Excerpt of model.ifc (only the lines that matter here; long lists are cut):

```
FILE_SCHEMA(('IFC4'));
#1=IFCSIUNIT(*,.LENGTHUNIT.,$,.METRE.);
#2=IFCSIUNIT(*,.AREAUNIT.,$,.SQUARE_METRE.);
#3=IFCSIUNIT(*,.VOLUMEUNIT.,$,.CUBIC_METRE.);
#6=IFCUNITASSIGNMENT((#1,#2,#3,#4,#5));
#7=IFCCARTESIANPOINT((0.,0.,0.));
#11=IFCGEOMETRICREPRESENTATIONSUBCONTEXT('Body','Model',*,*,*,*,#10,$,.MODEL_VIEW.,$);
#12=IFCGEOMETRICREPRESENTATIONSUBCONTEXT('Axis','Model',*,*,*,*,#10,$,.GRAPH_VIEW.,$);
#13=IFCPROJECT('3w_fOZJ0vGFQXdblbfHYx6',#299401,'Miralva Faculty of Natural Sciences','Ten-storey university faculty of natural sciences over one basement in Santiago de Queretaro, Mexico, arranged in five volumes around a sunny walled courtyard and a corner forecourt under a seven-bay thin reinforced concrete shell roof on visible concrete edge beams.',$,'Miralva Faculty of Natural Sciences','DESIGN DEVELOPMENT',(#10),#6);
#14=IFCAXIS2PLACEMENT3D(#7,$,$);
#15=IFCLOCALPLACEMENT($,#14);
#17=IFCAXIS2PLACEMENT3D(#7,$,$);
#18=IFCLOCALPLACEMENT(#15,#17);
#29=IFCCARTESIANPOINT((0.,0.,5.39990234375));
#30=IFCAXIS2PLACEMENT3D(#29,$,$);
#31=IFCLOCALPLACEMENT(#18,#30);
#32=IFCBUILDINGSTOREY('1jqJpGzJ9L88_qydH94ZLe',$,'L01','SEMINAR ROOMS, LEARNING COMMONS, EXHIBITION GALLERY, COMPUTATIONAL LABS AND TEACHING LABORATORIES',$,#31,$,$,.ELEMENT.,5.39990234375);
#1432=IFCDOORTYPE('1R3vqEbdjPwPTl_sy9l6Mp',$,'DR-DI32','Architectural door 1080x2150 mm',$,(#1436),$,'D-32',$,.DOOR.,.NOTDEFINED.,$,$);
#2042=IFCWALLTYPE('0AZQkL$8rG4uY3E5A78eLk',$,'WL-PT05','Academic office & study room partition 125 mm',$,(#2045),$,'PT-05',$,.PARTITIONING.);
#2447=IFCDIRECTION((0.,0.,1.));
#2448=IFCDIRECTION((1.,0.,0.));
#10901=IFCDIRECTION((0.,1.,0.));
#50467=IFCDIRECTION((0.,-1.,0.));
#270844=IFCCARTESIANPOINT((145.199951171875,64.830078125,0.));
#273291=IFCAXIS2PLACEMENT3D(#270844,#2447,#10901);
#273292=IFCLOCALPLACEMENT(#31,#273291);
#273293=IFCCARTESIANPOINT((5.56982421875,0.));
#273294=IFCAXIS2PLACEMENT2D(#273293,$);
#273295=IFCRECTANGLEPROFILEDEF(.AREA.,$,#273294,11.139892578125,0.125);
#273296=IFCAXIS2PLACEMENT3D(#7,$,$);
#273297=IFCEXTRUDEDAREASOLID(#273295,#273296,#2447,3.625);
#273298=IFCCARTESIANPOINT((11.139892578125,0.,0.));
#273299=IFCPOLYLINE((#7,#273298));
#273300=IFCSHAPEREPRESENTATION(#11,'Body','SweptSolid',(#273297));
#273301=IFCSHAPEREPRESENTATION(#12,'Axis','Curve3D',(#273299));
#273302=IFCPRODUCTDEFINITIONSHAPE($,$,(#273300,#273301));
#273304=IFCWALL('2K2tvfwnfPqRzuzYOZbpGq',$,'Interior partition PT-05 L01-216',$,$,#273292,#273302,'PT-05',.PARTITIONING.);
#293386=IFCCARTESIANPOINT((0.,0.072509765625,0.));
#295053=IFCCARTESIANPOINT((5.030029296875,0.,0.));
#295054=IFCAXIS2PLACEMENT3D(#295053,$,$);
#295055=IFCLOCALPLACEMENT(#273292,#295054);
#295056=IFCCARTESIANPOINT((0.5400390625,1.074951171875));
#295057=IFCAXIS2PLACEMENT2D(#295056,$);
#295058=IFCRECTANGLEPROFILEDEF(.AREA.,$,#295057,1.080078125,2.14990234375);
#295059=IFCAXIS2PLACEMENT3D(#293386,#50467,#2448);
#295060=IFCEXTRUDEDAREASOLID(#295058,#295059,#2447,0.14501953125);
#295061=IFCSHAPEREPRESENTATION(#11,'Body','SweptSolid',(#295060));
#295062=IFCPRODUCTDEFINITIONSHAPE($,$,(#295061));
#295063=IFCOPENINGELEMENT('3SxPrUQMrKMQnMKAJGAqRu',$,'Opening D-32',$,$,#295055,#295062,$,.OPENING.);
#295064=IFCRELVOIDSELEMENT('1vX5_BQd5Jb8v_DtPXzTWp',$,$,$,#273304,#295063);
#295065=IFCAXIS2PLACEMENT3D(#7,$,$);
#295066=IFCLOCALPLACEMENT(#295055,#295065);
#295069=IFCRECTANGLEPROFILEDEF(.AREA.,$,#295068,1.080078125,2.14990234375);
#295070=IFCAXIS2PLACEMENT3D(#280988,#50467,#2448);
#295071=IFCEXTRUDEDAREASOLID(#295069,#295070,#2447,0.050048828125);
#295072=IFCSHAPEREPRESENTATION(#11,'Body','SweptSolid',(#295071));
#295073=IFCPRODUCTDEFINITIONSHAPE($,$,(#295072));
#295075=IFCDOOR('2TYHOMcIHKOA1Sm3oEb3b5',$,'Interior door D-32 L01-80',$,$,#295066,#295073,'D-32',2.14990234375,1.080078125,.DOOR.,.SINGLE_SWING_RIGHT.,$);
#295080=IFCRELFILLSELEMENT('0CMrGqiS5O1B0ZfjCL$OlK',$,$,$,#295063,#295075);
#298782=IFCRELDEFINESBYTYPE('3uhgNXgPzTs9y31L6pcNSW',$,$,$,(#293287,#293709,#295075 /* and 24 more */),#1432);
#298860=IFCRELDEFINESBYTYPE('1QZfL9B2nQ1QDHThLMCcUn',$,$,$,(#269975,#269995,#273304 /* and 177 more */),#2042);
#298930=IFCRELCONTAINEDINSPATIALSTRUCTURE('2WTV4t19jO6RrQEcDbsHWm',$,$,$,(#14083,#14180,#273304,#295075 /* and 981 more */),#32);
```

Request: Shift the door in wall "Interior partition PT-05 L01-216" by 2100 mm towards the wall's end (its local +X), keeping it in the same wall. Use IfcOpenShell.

```python
import ifcopenshell
import ifcopenshell.api.geometry
import ifcopenshell.util.placement
import ifcopenshell.util.unit

model = ifcopenshell.open("model.ifc")
unit_scale = ifcopenshell.util.unit.calculate_unit_scale(model)

door = model.by_guid("2TYHOMcIHKOA1Sm3oEb3b5")
opening = door.FillsVoids[0].RelatingOpeningElement
wall = opening.VoidsElements[0].RelatingBuildingElement

wall_matrix = ifcopenshell.util.placement.get_local_placement(wall.ObjectPlacement)
shift = wall_matrix[:3, 0] * 2.1 / unit_scale
before = ifcopenshell.util.placement.get_local_placement(door.ObjectPlacement)[:3, 3].copy()

# The door is placed relative to its opening, so it follows when the opening moves.
matrix = ifcopenshell.util.placement.get_local_placement(opening.ObjectPlacement)
matrix[:3, 3] += shift
ifcopenshell.api.geometry.edit_object_placement(
    model, product=opening, matrix=matrix, is_si=False, should_transform_children=True
)

after = ifcopenshell.util.placement.get_local_placement(door.ObjectPlacement)[:3, 3]
print("door moved by", (after - before).round(3) + 0.0)

model.write("model_edited.ifc")
```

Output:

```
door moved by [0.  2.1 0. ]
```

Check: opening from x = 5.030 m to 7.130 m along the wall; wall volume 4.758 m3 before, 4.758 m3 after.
